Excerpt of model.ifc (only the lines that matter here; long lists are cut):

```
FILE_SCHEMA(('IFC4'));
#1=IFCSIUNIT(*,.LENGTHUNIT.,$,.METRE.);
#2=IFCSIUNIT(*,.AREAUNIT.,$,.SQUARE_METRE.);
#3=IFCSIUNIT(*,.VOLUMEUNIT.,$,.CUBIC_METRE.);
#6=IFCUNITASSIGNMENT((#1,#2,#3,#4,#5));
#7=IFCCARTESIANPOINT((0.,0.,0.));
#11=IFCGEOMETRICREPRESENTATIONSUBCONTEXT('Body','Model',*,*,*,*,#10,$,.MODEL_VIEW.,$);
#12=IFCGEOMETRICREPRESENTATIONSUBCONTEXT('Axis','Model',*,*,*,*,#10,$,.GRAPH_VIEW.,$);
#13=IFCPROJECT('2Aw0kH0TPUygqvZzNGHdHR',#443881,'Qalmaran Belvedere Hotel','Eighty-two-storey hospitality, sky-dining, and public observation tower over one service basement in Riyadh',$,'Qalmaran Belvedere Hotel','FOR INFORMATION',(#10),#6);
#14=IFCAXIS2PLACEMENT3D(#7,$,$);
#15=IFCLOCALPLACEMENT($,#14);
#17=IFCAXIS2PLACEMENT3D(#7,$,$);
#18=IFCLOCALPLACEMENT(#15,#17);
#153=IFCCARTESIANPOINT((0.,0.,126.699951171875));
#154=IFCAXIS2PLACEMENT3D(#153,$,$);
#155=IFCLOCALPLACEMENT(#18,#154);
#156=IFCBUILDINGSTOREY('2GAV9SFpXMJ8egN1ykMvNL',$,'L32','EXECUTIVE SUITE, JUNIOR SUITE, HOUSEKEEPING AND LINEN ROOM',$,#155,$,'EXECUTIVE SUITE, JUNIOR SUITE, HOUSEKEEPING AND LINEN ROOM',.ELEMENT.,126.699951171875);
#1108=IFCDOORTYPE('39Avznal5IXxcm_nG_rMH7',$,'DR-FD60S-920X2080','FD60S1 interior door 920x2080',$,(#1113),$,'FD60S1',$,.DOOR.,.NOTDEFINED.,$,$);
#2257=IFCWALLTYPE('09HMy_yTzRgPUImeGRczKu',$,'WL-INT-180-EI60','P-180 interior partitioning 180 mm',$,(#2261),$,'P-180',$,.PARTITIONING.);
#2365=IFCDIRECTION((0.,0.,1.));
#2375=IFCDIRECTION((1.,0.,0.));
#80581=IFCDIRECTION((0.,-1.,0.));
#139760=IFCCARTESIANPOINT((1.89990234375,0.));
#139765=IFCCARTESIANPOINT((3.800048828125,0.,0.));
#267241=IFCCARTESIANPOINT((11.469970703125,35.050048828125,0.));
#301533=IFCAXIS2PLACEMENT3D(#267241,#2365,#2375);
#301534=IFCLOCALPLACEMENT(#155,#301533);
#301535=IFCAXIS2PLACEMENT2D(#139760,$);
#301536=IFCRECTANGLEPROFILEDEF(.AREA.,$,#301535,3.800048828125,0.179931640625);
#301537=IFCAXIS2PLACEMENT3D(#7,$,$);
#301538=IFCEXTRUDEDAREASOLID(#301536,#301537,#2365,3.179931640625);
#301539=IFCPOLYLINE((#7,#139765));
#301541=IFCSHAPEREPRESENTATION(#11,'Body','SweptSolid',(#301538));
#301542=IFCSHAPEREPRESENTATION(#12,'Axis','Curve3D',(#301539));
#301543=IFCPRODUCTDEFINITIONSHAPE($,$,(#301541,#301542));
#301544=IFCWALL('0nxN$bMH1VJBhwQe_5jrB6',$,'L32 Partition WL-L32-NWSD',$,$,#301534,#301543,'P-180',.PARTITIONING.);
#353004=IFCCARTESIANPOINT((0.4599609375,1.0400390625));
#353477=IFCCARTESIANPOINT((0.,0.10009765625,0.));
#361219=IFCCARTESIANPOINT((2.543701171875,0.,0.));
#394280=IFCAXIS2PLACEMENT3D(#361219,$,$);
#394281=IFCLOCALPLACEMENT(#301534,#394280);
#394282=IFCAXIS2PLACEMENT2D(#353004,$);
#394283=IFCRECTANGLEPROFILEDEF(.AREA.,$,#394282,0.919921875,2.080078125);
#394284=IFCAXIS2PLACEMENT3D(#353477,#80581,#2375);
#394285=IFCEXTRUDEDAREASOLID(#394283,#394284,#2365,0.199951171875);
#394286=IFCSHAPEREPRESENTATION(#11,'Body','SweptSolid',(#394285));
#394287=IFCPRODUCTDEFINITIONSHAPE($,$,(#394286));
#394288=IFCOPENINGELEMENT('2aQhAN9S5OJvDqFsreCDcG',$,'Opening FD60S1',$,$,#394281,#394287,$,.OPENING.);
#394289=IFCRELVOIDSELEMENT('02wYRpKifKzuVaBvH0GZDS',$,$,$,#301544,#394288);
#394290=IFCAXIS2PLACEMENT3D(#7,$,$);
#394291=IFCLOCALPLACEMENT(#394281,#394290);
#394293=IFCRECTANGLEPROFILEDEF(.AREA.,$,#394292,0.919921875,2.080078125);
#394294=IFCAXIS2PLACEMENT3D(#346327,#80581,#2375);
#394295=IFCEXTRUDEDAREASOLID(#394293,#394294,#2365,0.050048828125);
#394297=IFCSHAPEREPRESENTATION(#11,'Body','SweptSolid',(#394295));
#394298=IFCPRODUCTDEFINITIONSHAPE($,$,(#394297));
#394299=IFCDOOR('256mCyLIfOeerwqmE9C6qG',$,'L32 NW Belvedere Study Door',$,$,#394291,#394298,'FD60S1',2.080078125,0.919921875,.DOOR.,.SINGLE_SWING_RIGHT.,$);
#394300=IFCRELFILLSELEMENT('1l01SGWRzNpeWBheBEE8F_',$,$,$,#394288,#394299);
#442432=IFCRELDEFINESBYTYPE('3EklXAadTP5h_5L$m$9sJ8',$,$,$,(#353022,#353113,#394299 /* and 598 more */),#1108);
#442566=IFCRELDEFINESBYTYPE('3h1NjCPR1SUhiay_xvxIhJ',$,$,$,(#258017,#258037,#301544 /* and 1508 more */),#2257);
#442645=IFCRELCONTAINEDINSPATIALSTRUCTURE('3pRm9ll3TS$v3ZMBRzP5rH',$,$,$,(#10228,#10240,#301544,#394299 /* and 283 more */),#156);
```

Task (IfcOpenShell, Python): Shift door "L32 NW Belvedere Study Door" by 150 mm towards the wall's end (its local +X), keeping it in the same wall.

```python
import ifcopenshell
import ifcopenshell.api.geometry
import ifcopenshell.util.placement
import ifcopenshell.util.unit

model = ifcopenshell.open("model.ifc")
unit_scale = ifcopenshell.util.unit.calculate_unit_scale(model)

door = model.by_guid("256mCyLIfOeerwqmE9C6qG")
opening = door.FillsVoids[0].RelatingOpeningElement
wall = opening.VoidsElements[0].RelatingBuildingElement

wall_matrix = ifcopenshell.util.placement.get_local_placement(wall.ObjectPlacement)
shift = wall_matrix[:3, 0] * 0.15 / unit_scale
before = ifcopenshell.util.placement.get_local_placement(door.ObjectPlacement)[:3, 3].copy()

# The door is placed relative to its opening, so it follows when the opening moves.
matrix = ifcopenshell.util.placement.get_local_placement(opening.ObjectPlacement)
matrix[:3, 3] += shift
ifcopenshell.api.geometry.edit_object_placement(
    model, product=opening, matrix=matrix, is_si=False, should_transform_children=True
)

after = ifcopenshell.util.placement.get_local_placement(door.ObjectPlacement)[:3, 3]
print("door moved by", (after - before).round(3) + 0.0)

model.write("model-out.ifc")
```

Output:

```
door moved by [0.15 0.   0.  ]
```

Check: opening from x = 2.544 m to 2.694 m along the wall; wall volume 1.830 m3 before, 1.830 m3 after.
